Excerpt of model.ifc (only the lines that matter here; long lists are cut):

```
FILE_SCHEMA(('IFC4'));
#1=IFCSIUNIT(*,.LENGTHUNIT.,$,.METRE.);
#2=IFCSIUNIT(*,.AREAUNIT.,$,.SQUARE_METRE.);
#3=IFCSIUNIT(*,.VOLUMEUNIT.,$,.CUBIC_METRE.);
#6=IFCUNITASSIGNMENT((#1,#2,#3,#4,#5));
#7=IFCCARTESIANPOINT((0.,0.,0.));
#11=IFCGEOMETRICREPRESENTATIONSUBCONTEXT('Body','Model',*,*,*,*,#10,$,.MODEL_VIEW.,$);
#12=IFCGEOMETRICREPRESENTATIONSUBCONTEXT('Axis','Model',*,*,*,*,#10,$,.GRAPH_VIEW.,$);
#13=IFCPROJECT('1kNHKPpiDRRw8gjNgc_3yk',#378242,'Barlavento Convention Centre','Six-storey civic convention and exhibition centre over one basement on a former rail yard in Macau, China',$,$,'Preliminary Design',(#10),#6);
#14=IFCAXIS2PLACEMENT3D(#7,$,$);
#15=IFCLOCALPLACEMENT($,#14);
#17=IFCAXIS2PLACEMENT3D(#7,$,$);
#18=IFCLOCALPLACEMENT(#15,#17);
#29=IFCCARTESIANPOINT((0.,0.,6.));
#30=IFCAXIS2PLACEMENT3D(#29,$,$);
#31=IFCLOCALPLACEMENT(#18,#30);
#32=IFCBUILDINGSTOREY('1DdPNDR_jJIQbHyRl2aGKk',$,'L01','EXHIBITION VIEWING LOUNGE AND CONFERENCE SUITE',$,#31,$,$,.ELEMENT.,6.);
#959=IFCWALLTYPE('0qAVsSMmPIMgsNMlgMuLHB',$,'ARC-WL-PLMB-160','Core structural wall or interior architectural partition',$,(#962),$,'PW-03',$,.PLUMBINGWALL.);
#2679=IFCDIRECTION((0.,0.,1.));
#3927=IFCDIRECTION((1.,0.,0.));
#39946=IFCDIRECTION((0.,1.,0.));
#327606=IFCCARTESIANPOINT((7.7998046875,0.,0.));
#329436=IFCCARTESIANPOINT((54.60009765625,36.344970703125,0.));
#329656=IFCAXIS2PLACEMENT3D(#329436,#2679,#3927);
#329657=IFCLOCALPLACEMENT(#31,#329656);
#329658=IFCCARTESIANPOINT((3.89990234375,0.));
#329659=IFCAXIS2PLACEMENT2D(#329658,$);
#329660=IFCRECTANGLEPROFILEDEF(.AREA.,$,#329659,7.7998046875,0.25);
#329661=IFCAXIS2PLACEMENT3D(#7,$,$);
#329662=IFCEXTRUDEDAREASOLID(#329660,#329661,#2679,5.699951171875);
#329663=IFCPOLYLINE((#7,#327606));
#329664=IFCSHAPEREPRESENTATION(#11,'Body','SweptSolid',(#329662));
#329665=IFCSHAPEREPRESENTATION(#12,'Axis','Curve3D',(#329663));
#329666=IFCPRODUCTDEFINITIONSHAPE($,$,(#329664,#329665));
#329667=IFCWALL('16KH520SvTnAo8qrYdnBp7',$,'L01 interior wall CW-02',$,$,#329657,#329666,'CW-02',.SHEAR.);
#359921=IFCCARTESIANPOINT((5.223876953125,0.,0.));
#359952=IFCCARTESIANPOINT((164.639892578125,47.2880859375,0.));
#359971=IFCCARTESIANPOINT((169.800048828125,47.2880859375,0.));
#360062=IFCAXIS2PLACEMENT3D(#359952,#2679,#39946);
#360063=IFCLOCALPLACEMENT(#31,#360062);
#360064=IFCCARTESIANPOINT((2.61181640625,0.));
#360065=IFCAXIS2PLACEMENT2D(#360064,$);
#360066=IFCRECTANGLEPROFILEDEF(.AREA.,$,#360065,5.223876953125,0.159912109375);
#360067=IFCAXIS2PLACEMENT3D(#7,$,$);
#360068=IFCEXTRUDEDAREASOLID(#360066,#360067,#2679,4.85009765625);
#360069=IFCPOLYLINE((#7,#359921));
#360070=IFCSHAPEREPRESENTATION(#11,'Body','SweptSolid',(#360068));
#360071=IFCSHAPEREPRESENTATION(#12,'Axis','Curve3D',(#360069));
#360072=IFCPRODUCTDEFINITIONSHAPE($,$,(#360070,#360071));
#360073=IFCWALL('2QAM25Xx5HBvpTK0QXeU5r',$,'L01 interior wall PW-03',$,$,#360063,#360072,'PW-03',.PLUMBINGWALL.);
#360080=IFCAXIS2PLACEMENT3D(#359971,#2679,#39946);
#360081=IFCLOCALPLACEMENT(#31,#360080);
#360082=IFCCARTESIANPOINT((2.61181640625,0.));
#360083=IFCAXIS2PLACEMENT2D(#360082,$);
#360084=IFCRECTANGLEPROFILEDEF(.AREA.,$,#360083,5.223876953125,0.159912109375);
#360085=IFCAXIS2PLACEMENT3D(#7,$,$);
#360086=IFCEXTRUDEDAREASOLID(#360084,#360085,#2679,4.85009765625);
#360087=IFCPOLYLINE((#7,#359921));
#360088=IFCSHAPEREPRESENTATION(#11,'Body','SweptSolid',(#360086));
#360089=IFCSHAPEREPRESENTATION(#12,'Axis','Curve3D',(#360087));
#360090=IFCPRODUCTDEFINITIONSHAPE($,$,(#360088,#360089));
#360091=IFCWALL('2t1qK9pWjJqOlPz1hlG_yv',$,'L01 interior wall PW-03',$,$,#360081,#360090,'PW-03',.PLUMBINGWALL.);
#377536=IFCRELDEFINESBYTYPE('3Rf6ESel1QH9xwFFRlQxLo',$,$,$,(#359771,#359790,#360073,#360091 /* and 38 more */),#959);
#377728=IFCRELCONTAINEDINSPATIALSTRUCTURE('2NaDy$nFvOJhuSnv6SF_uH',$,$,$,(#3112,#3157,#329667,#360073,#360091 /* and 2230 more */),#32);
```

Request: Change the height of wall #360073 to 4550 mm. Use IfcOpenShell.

```python
import ifcopenshell
import ifcopenshell.geom
import ifcopenshell.util.representation
import ifcopenshell.util.shape

model = ifcopenshell.open("model.ifc")
settings = ifcopenshell.geom.settings()


def volume(element):
    """Net volume in cubic metres, openings subtracted."""
    shape = ifcopenshell.geom.create_shape(settings, element)
    return ifcopenshell.util.shape.get_volume(shape.geometry)


wall = model.by_guid("2QAM25Xx5HBvpTK0QXeU5r")
before = volume(wall)

body = ifcopenshell.util.representation.get_representation(wall, "Model", "Body")
solid = body.Items[0]
old_height = solid.Depth
solid.Depth = 4.55
after = volume(wall)

print(f"height {old_height:g} -> {solid.Depth:g}, volume {before:.3f} -> {after:.3f} m3")

model.write("model_rev.ifc")
```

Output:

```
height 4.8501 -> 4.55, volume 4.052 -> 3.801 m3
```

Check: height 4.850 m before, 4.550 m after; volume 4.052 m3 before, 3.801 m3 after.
